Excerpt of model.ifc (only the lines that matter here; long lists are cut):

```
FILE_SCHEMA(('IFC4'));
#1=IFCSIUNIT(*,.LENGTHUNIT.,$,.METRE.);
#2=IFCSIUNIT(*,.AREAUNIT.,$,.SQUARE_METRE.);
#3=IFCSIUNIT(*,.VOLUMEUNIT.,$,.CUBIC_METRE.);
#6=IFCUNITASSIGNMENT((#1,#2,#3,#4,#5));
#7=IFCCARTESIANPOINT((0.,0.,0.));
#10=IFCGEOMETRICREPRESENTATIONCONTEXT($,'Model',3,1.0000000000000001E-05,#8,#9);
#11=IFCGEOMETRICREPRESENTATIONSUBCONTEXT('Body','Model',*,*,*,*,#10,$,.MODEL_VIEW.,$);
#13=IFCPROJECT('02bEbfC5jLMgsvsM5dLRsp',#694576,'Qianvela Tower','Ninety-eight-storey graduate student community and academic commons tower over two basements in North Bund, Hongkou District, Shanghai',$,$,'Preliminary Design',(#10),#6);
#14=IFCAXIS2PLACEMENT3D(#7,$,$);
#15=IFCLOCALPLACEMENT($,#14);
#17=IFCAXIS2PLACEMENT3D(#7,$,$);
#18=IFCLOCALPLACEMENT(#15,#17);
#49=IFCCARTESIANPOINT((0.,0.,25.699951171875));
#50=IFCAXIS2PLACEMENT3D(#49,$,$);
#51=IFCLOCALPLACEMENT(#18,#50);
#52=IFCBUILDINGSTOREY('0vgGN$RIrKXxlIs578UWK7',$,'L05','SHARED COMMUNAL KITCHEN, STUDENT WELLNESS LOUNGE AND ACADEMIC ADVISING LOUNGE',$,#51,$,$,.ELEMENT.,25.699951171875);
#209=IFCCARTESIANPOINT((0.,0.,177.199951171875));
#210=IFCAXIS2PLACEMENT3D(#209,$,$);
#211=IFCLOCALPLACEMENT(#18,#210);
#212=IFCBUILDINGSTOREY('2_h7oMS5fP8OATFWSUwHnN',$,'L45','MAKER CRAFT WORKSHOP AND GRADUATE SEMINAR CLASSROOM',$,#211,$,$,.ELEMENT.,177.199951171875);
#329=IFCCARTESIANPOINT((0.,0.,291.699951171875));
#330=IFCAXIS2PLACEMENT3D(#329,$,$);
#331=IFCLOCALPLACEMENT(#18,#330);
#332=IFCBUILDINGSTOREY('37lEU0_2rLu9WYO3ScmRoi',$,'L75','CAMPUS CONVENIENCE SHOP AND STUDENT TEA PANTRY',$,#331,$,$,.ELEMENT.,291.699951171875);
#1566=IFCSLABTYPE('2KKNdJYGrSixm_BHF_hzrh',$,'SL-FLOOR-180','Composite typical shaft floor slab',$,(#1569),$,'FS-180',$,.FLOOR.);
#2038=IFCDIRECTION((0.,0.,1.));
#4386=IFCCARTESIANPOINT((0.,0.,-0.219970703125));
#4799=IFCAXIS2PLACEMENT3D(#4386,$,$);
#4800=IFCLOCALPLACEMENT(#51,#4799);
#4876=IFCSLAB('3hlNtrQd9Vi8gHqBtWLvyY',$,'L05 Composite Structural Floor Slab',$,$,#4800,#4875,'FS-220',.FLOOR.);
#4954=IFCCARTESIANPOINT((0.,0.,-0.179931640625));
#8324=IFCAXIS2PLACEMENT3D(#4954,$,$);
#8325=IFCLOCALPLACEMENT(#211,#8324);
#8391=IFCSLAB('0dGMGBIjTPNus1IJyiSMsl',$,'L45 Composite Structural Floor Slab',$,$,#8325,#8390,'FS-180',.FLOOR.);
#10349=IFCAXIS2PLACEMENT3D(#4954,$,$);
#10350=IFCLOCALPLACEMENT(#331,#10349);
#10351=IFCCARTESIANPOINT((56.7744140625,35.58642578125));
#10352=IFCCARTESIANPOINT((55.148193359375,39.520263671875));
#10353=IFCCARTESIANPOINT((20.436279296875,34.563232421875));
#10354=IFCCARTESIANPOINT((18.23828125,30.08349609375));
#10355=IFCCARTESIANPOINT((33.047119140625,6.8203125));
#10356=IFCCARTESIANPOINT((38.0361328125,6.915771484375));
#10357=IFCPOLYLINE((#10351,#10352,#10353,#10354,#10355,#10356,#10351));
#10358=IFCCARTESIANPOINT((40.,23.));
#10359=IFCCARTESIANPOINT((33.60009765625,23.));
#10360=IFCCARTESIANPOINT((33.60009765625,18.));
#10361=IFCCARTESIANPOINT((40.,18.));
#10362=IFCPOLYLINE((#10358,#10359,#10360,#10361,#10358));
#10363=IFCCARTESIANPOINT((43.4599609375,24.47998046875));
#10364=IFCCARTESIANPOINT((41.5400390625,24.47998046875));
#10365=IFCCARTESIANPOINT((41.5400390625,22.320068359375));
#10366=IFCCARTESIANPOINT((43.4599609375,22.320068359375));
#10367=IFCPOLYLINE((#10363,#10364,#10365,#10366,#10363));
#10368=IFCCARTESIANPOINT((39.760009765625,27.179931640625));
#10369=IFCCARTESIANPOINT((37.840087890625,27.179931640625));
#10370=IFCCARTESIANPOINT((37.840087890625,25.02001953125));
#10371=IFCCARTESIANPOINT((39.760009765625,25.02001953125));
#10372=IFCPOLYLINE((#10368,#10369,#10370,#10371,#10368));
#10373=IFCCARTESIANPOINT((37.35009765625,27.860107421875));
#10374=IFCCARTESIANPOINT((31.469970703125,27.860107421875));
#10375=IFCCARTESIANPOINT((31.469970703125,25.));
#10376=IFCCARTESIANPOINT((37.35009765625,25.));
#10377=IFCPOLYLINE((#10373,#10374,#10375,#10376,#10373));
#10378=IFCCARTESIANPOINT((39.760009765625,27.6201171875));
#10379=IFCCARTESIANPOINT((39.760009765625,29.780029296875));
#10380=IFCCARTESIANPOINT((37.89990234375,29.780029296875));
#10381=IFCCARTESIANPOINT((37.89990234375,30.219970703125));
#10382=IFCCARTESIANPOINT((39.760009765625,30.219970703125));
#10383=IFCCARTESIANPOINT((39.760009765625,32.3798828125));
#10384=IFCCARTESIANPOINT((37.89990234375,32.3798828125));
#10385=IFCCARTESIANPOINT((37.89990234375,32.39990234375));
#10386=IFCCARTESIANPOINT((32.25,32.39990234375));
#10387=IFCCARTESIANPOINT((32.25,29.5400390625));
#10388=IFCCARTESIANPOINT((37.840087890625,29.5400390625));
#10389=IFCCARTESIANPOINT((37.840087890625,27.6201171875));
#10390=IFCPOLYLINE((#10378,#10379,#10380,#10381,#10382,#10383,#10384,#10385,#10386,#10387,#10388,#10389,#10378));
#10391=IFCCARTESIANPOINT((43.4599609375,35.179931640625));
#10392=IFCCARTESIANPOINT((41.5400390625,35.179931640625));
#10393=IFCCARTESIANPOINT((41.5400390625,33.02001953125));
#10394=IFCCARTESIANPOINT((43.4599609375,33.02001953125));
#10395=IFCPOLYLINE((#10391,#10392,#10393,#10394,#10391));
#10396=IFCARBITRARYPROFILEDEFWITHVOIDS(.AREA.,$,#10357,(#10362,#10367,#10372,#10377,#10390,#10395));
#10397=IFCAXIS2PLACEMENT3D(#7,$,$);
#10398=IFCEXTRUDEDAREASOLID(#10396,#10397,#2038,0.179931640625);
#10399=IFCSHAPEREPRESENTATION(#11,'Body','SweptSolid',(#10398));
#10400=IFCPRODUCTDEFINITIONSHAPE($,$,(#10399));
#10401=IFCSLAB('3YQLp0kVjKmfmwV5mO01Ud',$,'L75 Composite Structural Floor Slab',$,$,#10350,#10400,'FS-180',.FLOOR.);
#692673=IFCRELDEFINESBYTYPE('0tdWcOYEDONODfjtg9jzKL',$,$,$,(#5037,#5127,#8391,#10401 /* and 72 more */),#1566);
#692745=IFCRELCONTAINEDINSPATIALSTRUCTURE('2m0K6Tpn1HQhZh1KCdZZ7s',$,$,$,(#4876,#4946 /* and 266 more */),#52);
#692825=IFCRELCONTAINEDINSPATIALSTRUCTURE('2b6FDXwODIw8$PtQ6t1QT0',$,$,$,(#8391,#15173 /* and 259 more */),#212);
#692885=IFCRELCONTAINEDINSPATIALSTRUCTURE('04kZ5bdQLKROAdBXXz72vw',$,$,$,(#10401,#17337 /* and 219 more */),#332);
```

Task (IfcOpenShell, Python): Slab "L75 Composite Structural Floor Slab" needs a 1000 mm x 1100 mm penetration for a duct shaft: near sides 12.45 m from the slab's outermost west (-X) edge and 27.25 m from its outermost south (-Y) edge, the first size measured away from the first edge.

```python
import numpy as np
import ifcopenshell
import ifcopenshell.api.feature
import ifcopenshell.api.geometry
import ifcopenshell.api.root
import ifcopenshell.geom
import ifcopenshell.util.placement
import ifcopenshell.util.representation
import ifcopenshell.util.shape
import ifcopenshell.util.unit

model = ifcopenshell.open("model.ifc")
unit_scale = ifcopenshell.util.unit.calculate_unit_scale(model)
settings = ifcopenshell.geom.settings()


def volume(element):
    """Net volume in cubic metres, openings subtracted."""
    shape = ifcopenshell.geom.create_shape(settings, element)
    return ifcopenshell.util.shape.get_volume(shape.geometry)


slab = model.by_id(10401)
before = volume(slab)

# Extent in the slab's own axes, in metres. The edges named are its -X and -Y sides.
slab_shape = ifcopenshell.geom.create_shape(settings, slab)
vertices = ifcopenshell.util.shape.get_vertices(slab_shape.geometry)
x_min, y_min, bottom = vertices.min(axis=0)
top = vertices[:, 2].max()

opening = ifcopenshell.api.root.create_entity(model, ifc_class="IfcOpeningElement", name="Duct shaft opening", predefined_type="OPENING")
context = ifcopenshell.util.representation.get_context(model, "Model", "Body", "MODEL_VIEW")
width, depth = 1, 1.1
outline = [(0.0, 0.0), (width, 0.0), (width, depth), (0.0, depth), (0.0, 0.0)]
# Overshoot both faces by 50 mm so the cut is clean.
shape = ifcopenshell.api.geometry.add_slab_representation(
    model, context=context, depth=top - bottom + 0.1, polyline=outline
)
ifcopenshell.api.geometry.assign_representation(model, product=opening, representation=shape)

matrix = ifcopenshell.util.placement.get_local_placement(slab.ObjectPlacement)
matrix[:, 3] = matrix @ np.append(np.array([x_min + 12.45, y_min + 27.25, bottom - 0.05]) / unit_scale, 1.0)
ifcopenshell.api.geometry.edit_object_placement(model, product=opening, matrix=matrix, is_si=False)
ifcopenshell.api.feature.add_feature(model, feature=opening, element=slab)

after = volume(slab)

print(f"slab volume {before:.3f} -> {after:.3f} m3")

model.write("model-out.ifc")
```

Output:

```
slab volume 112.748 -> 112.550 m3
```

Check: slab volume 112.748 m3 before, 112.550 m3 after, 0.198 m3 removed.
